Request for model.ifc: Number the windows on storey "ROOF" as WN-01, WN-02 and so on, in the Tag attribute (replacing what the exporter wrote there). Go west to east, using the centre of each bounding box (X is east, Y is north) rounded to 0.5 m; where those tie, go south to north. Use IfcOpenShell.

First a look at what the model holds.

```python
import ifcopenshell
import ifcopenshell.util.element
import ifcopenshell.util.placement

model = ifcopenshell.open("model.ifc")
print(model.schema)
storey = next(s for s in model.by_type("IfcBuildingStorey") if s.Name == "ROOF")
windows = [e for e in ifcopenshell.util.element.get_decomposition(storey) if e.is_a("IfcWindow")]
for e in sorted(windows, key=lambda e: e.id()):
    origin = ifcopenshell.util.placement.get_local_placement(e.ObjectPlacement)[:3, 3]
    print(e.id(), e.Tag, e.Name, origin.round(2) + 0.0, sep=" | ")
```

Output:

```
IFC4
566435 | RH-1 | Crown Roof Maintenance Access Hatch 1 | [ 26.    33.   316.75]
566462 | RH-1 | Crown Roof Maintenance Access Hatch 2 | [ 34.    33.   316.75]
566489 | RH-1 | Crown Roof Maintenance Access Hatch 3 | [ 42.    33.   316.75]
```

```python
import ifcopenshell
import ifcopenshell.geom
import ifcopenshell.util.element
import ifcopenshell.util.shape

model = ifcopenshell.open("model.ifc")
settings = ifcopenshell.geom.settings()
settings.set("use-world-coords", True)


def centre(element):
    shape = ifcopenshell.geom.create_shape(settings, element)
    return ifcopenshell.util.shape.get_bbox_centroid(shape.geometry)


storey = next(s for s in model.by_type("IfcBuildingStorey") if s.Name == "ROOF")
windows = [e for e in ifcopenshell.util.element.get_decomposition(storey) if e.is_a("IfcWindow")]

# Insertion points can sit at a corner or the storey origin, so sort by the geometry (in metres).
centres = {e: centre(e) for e in windows}
windows.sort(key=lambda e: (round(centres[e][0] / 0.5), centres[e][1]))

for i, e in enumerate(windows, start=1):
    number = f"WN-{i:02d}"
    e.Tag = number
    print(e.id(), number)

model.write("model_v2.ifc")
```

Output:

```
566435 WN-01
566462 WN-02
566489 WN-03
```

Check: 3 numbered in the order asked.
